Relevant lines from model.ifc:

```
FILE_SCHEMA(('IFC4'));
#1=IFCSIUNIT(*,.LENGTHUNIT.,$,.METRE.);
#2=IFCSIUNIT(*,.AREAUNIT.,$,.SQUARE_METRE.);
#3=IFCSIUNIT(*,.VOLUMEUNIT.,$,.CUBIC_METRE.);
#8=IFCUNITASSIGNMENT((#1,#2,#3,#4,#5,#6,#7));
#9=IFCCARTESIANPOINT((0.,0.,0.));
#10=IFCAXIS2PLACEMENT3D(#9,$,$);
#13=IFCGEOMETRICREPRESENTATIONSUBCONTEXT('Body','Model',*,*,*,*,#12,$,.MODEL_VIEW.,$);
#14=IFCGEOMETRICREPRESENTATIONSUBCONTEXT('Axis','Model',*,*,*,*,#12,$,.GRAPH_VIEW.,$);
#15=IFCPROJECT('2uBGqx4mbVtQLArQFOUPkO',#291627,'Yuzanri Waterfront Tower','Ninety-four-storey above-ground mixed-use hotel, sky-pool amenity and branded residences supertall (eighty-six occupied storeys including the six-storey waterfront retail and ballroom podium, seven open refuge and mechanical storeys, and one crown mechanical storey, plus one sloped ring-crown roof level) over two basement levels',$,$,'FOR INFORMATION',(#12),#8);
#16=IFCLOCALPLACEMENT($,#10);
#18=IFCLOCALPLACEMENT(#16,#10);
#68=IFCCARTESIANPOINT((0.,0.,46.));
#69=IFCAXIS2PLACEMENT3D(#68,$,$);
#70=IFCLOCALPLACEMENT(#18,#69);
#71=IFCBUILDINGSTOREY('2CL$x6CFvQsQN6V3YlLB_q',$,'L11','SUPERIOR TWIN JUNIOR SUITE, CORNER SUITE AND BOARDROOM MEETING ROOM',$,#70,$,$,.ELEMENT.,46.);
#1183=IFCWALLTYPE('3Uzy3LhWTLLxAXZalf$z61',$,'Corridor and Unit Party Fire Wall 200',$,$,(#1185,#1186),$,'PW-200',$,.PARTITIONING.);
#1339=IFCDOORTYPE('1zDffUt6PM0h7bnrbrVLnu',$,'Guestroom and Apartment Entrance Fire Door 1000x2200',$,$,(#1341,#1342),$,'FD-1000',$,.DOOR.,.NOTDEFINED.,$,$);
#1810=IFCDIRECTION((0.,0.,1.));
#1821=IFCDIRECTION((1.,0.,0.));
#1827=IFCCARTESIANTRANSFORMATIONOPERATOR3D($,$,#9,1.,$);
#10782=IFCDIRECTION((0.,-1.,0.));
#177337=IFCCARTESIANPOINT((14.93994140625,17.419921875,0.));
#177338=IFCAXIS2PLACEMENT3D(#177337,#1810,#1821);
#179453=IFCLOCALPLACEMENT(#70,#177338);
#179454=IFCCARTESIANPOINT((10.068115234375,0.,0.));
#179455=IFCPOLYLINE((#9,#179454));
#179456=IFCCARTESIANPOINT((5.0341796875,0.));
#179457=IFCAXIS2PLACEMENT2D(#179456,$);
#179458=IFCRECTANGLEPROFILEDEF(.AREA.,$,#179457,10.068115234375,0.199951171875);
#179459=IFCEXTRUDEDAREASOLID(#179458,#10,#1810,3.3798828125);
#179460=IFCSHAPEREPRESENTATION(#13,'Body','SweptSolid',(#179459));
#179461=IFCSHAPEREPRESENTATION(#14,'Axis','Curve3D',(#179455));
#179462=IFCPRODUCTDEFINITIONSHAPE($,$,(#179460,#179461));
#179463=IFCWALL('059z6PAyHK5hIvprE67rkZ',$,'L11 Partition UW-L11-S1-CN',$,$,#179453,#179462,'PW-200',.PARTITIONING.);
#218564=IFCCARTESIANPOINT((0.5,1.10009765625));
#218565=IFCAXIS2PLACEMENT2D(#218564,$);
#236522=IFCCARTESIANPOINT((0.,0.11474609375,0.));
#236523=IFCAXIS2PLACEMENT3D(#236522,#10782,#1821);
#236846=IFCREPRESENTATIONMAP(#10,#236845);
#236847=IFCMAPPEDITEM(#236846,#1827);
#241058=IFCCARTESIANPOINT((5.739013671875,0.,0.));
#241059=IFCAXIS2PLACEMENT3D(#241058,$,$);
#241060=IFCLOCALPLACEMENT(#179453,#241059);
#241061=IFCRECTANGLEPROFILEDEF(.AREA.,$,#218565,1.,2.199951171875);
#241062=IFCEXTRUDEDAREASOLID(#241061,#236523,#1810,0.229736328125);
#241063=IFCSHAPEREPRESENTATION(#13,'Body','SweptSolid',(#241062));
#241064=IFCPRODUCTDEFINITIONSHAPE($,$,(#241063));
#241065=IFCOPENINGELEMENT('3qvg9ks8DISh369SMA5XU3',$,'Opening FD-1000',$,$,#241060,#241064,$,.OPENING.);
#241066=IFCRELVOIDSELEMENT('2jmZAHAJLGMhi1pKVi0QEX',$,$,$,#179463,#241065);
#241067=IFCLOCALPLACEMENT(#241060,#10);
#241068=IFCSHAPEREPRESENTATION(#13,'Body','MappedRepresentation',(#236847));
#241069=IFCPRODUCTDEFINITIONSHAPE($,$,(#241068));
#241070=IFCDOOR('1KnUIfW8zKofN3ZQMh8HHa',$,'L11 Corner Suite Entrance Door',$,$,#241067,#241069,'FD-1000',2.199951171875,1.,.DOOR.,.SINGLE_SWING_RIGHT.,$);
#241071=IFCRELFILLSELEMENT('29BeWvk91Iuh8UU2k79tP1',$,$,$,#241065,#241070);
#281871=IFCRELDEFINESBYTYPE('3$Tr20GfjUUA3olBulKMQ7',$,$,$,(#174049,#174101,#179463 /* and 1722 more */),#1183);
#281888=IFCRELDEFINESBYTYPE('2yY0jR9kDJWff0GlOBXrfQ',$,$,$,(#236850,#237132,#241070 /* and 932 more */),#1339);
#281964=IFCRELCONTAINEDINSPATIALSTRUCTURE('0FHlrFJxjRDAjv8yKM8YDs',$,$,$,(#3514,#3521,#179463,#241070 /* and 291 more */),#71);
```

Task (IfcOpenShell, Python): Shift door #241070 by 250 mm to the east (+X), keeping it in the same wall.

```python
import ifcopenshell
import ifcopenshell.api.geometry
import ifcopenshell.util.placement
import ifcopenshell.util.unit

model = ifcopenshell.open("model.ifc")
unit_scale = ifcopenshell.util.unit.calculate_unit_scale(model)

door = model.by_guid("1KnUIfW8zKofN3ZQMh8HHa")
opening = door.FillsVoids[0].RelatingOpeningElement
wall = opening.VoidsElements[0].RelatingBuildingElement

wall_matrix = ifcopenshell.util.placement.get_local_placement(wall.ObjectPlacement)
shift = wall_matrix[:3, 0] * 0.25 / unit_scale
before = ifcopenshell.util.placement.get_local_placement(door.ObjectPlacement)[:3, 3].copy()

# The door is placed relative to its opening, so it follows when the opening moves.
matrix = ifcopenshell.util.placement.get_local_placement(opening.ObjectPlacement)
matrix[:3, 3] += shift
ifcopenshell.api.geometry.edit_object_placement(
    model, product=opening, matrix=matrix, is_si=False, should_transform_children=True
)

after = ifcopenshell.util.placement.get_local_placement(door.ObjectPlacement)[:3, 3]
print("door moved by", (after - before).round(3) + 0.0)

model.write("model_rev.ifc")
```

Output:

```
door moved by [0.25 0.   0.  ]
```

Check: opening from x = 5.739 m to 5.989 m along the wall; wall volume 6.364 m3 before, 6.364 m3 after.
